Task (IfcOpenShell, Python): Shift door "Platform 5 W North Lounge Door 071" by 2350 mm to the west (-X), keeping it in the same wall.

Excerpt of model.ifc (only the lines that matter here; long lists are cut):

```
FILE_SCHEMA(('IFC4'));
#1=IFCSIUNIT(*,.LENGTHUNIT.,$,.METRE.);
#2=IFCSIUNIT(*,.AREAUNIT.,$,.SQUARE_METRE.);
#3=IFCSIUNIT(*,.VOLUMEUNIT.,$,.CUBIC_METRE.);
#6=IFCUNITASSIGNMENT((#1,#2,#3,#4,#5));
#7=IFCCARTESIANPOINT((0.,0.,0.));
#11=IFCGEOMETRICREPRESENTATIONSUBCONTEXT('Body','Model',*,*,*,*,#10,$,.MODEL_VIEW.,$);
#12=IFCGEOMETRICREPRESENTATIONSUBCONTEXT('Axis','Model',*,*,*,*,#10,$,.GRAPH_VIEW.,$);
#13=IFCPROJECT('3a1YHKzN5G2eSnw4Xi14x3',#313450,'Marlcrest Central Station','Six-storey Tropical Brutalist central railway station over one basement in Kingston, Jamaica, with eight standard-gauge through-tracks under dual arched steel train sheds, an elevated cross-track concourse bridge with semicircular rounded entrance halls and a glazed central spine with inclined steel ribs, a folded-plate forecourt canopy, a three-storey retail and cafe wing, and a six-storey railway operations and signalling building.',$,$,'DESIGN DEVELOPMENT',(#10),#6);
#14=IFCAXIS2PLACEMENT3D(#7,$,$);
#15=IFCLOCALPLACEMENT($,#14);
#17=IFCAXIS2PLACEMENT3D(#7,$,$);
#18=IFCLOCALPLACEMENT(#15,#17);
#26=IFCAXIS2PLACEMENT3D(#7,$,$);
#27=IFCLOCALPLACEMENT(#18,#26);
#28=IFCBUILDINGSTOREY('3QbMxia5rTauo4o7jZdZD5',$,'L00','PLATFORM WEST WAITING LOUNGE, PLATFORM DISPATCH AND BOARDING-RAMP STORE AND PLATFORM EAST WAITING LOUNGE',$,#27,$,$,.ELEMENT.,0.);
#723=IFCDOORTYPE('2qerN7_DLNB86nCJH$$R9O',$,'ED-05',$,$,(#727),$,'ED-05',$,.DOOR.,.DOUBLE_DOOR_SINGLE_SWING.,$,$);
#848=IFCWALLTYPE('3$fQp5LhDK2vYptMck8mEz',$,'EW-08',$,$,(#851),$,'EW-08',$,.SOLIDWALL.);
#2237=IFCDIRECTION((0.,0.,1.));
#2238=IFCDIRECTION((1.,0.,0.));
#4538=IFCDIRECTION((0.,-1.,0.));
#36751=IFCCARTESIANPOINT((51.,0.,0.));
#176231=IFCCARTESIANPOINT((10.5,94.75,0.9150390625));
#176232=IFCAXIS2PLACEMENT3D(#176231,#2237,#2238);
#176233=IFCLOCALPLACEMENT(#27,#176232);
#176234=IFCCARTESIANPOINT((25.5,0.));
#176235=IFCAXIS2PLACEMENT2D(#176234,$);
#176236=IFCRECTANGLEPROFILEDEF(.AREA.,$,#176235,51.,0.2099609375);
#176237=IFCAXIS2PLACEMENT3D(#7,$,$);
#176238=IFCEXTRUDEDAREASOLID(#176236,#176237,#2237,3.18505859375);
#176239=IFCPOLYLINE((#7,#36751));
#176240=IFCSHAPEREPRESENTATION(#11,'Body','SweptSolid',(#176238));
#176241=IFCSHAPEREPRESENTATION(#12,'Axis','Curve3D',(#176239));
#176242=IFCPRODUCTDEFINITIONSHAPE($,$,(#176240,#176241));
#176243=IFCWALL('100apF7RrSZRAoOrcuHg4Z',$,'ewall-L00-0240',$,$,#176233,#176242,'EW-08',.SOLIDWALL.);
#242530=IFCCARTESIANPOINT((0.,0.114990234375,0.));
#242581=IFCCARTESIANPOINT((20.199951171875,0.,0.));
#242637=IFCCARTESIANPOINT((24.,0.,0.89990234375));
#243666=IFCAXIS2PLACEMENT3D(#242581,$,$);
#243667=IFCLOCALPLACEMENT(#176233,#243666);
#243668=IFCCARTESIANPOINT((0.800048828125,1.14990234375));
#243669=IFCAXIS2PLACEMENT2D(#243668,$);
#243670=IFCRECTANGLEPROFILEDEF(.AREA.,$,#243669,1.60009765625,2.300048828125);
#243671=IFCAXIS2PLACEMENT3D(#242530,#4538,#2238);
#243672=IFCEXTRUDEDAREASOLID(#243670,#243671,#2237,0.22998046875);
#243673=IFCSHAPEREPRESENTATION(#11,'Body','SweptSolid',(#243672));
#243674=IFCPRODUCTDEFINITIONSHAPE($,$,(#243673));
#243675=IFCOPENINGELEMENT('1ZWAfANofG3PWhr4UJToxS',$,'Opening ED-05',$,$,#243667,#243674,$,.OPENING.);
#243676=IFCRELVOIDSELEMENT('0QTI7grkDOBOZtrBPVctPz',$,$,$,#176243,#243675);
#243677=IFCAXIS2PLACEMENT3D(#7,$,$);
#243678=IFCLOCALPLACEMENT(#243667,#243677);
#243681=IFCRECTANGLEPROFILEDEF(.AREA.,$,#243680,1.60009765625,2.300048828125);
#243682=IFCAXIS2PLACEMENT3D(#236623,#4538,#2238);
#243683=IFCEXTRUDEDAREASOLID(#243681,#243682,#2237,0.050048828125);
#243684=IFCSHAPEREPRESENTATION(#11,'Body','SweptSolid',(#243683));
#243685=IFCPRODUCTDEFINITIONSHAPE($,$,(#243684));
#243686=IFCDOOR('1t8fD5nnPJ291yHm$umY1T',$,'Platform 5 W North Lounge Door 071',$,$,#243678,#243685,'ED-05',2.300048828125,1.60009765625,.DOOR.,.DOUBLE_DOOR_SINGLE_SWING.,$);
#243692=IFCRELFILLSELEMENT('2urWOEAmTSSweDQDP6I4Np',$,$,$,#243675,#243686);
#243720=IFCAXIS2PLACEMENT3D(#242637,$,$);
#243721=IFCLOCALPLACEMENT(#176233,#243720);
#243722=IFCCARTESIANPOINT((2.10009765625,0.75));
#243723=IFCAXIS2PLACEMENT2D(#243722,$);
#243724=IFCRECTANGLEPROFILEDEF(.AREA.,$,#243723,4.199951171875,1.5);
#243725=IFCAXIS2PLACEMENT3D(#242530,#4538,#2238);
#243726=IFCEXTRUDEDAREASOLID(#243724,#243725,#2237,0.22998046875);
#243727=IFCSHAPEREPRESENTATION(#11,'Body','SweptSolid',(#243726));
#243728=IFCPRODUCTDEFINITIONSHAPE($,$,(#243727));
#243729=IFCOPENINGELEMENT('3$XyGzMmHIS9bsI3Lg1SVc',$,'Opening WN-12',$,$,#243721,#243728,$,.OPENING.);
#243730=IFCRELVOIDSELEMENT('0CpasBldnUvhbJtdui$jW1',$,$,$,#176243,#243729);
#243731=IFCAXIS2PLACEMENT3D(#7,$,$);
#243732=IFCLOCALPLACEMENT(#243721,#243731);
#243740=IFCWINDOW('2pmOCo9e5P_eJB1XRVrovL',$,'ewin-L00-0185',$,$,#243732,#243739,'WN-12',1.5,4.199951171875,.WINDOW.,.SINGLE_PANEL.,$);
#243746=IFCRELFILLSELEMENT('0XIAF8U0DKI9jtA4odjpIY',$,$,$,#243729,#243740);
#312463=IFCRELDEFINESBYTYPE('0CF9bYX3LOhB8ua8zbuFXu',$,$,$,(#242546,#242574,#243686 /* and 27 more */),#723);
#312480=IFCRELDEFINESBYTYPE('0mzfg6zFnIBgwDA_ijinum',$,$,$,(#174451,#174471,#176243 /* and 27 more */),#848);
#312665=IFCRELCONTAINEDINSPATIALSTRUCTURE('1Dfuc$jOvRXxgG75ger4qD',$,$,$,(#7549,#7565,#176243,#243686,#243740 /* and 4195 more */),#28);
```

```python
import ifcopenshell
import ifcopenshell.api.geometry
import ifcopenshell.util.placement

model = ifcopenshell.open("model.ifc")

door = model.by_guid("1t8fD5nnPJ291yHm$umY1T")
opening = door.FillsVoids[0].RelatingOpeningElement
wall = opening.VoidsElements[0].RelatingBuildingElement

wall_matrix = ifcopenshell.util.placement.get_local_placement(wall.ObjectPlacement)
shift = wall_matrix[:3, 0] * -2.35
before = ifcopenshell.util.placement.get_local_placement(door.ObjectPlacement)[:3, 3].copy()

# The door is placed relative to its opening, so it follows when the opening moves.
matrix = ifcopenshell.util.placement.get_local_placement(opening.ObjectPlacement)
matrix[:3, 3] += shift
ifcopenshell.api.geometry.edit_object_placement(
    model, product=opening, matrix=matrix, is_si=False, should_transform_children=True
)

after = ifcopenshell.util.placement.get_local_placement(door.ObjectPlacement)[:3, 3]
print("door moved by", (after - before).round(3) + 0.0)

model.write("model-out.ifc")
```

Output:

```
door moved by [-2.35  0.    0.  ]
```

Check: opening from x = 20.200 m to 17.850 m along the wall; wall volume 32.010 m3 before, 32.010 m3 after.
